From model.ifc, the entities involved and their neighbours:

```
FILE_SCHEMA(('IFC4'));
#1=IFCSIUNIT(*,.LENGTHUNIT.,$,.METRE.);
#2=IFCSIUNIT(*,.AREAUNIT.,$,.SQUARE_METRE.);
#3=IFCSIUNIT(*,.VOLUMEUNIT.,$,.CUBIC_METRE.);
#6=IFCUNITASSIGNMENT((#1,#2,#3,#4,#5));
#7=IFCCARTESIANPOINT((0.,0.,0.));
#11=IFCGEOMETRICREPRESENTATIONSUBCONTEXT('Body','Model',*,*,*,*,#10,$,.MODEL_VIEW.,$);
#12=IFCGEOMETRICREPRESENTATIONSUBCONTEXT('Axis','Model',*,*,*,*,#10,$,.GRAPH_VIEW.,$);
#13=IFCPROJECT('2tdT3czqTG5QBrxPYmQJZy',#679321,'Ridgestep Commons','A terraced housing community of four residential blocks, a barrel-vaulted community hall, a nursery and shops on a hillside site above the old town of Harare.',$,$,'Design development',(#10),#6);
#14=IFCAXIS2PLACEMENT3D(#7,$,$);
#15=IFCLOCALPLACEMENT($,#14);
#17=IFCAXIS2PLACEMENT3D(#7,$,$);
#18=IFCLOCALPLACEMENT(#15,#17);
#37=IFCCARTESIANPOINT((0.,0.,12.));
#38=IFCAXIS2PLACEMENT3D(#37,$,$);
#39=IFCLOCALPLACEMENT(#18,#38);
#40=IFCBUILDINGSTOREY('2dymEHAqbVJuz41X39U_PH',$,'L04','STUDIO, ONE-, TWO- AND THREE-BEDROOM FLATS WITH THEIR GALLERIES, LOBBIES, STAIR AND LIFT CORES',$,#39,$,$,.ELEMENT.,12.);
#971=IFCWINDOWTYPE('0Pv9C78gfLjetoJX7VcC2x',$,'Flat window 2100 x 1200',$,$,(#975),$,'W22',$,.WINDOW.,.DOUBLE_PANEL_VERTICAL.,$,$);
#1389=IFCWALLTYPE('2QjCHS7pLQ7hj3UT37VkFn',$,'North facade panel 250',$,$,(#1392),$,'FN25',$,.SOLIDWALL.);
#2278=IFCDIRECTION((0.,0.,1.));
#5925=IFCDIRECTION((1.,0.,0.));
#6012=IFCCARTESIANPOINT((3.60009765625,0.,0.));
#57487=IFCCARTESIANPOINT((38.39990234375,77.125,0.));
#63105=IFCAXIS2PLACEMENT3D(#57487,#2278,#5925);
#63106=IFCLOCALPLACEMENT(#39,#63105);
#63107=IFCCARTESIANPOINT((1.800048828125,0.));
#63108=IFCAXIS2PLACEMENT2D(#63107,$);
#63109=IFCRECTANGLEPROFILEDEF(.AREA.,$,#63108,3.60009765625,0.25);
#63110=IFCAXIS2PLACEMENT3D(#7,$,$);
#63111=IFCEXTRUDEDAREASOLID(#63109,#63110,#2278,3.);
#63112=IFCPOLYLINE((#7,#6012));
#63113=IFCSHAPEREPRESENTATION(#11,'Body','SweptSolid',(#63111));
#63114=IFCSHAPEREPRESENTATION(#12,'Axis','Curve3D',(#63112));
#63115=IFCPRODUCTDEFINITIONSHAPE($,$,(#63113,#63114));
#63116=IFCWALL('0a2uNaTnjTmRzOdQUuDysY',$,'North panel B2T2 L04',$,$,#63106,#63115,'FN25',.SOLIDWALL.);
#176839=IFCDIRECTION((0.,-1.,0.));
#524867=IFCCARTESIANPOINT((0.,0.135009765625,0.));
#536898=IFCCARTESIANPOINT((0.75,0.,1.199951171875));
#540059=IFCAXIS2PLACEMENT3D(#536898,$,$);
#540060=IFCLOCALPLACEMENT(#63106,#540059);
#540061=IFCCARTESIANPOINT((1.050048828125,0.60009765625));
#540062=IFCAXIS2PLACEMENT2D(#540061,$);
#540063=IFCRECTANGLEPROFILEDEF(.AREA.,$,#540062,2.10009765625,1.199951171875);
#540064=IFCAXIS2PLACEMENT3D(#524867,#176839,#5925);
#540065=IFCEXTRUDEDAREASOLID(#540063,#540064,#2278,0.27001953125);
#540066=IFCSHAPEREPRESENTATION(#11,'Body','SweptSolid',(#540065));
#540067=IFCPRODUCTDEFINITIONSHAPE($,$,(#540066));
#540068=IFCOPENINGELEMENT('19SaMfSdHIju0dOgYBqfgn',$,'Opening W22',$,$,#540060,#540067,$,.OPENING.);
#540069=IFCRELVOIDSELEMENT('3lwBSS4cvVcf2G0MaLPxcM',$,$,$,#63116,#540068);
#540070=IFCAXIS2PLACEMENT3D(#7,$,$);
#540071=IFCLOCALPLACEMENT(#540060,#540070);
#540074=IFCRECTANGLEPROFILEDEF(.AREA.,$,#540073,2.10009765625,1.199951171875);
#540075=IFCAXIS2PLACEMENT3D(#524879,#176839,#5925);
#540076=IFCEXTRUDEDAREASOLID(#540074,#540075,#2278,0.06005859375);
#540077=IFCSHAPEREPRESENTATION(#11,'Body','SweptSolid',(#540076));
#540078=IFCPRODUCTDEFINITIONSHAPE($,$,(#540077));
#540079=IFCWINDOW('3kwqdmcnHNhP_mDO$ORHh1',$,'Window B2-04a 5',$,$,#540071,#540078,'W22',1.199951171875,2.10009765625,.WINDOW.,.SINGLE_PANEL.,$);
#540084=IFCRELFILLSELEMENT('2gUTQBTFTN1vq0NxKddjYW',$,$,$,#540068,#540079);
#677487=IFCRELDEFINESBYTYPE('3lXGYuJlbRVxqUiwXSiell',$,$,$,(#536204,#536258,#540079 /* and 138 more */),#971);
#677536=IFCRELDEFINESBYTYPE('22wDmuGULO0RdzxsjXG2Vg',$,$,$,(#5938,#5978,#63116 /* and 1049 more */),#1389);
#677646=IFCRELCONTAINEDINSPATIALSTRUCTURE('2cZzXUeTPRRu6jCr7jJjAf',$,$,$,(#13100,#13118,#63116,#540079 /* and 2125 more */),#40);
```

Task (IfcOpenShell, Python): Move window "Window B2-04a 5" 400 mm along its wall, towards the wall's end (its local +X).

```python
import ifcopenshell
import ifcopenshell.api.geometry
import ifcopenshell.util.placement

model = ifcopenshell.open("model.ifc")

window = model.by_guid("3kwqdmcnHNhP_mDO$ORHh1")
opening = window.FillsVoids[0].RelatingOpeningElement
wall = opening.VoidsElements[0].RelatingBuildingElement

wall_matrix = ifcopenshell.util.placement.get_local_placement(wall.ObjectPlacement)
shift = wall_matrix[:3, 0] * 0.4
before = ifcopenshell.util.placement.get_local_placement(window.ObjectPlacement)[:3, 3].copy()

# The window is placed relative to its opening, so it follows when the opening moves.
matrix = ifcopenshell.util.placement.get_local_placement(opening.ObjectPlacement)
matrix[:3, 3] += shift
ifcopenshell.api.geometry.edit_object_placement(
    model, product=opening, matrix=matrix, is_si=False, should_transform_children=True
)

after = ifcopenshell.util.placement.get_local_placement(window.ObjectPlacement)[:3, 3]
print("window moved by", (after - before).round(3) + 0.0)

model.write("model-out.ifc")
```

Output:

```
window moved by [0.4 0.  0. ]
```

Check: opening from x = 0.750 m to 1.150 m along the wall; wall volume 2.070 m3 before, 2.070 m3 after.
